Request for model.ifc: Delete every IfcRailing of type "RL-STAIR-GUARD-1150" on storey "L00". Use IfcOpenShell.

First a look at what the model holds.

```python
import ifcopenshell
import ifcopenshell.util.element

model = ifcopenshell.open("model.ifc")
print(model.schema)
storey = next(s for s in model.by_type("IfcBuildingStorey") if s.Name == "L00")
railings = [e for e in ifcopenshell.util.element.get_decomposition(storey) if e.is_a("IfcRailing")]
seen = {}
for e in railings:
    element_type = ifcopenshell.util.element.get_type(e)
    name = element_type.Name if element_type not in (None, e) else None
    seen[name] = seen.get(name, 0) + 1
for name, count in sorted(seen.items(), key=str):
    print(count, "x", name)
```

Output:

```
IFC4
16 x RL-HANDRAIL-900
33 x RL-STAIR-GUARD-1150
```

```python
import ifcopenshell
import ifcopenshell.api.root
import ifcopenshell.util.element

model = ifcopenshell.open("model.ifc")

storey = next(s for s in model.by_type("IfcBuildingStorey") if s.Name == "L00")
railings = [e for e in ifcopenshell.util.element.get_decomposition(storey) if e.is_a("IfcRailing")]
targets = [e for e in railings if (t := ifcopenshell.util.element.get_type(e)) not in (None, e) and t.Name == "RL-STAIR-GUARD-1150"]

for e in targets:
    ifcopenshell.api.root.remove_product(model, product=e)
print(len(targets), "removed")

model.write("model_v2.ifc")
```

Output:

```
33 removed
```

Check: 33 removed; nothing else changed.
